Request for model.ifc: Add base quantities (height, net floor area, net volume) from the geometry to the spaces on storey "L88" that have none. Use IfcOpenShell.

First a look at what the model holds.

```python
import ifcopenshell
import ifcopenshell.util.element
import ifcopenshell.util.unit

model = ifcopenshell.open("model.ifc")
print(model.schema)
for unit_type in ("LENGTHUNIT", "AREAUNIT", "VOLUMEUNIT"):
    print(unit_type, ifcopenshell.util.unit.calculate_unit_scale(model, unit_type))
storey = next(s for s in model.by_type("IfcBuildingStorey") if s.Name == "L88")
spaces = [e for e in ifcopenshell.util.element.get_decomposition(storey) if e.is_a("IfcSpace")]
for e in sorted(spaces, key=lambda e: e.id()):
    print(e.id(), e.is_a(), e.Name, list(ifcopenshell.util.element.get_psets(e, qtos_only=True)), sep=" | ")
```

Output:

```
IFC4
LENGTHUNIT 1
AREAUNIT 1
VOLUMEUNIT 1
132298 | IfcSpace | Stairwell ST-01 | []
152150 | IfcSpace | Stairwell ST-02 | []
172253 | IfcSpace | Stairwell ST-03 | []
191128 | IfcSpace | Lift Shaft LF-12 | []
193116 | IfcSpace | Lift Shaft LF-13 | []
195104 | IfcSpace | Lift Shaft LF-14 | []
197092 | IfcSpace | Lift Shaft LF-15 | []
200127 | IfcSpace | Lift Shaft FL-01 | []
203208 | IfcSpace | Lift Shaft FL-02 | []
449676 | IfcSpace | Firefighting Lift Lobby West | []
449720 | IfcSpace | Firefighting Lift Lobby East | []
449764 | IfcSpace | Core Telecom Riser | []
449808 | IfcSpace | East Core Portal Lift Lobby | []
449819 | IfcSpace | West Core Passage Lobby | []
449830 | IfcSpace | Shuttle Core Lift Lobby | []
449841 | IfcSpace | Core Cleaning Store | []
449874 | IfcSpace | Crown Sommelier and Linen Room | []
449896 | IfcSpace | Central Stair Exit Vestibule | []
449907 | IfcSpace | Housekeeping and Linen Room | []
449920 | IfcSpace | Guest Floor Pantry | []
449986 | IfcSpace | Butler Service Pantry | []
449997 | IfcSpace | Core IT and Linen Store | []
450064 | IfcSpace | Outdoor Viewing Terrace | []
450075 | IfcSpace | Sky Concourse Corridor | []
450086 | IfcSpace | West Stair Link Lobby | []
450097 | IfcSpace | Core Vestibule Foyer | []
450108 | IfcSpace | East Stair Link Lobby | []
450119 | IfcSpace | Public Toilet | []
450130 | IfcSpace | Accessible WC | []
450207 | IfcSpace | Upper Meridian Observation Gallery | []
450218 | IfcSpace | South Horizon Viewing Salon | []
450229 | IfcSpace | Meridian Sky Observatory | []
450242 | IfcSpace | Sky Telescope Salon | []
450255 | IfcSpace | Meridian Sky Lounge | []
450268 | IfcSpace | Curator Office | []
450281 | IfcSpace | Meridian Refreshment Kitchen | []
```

```python
import ifcopenshell
import ifcopenshell.api.pset
import ifcopenshell.geom
import ifcopenshell.util.element
import ifcopenshell.util.shape
import ifcopenshell.util.unit

model = ifcopenshell.open("model.ifc")
unit_scale = ifcopenshell.util.unit.calculate_unit_scale(model)
area_scale = ifcopenshell.util.unit.calculate_unit_scale(model, "AREAUNIT")
volume_scale = ifcopenshell.util.unit.calculate_unit_scale(model, "VOLUMEUNIT")
settings = ifcopenshell.geom.settings()

storey = next(s for s in model.by_type("IfcBuildingStorey") if s.Name == "L88")
spaces = [e for e in ifcopenshell.util.element.get_decomposition(storey) if e.is_a("IfcSpace")]

for e in sorted(spaces, key=lambda e: e.id()):
    if ifcopenshell.util.element.get_psets(e, qtos_only=True, should_inherit=False):
        continue
    # Geometry comes back in metres, in the element's own axes.
    shape = ifcopenshell.geom.create_shape(settings, e)
    values = {
        "Height": ifcopenshell.util.shape.get_z(shape.geometry) / unit_scale,
        "NetFloorArea": ifcopenshell.util.shape.get_footprint_area(shape.geometry) / area_scale,
        "NetVolume": ifcopenshell.util.shape.get_volume(shape.geometry) / volume_scale,
    }
    qto = ifcopenshell.api.pset.add_qto(model, product=e, name="Qto_SpaceBaseQuantities")
    ifcopenshell.api.pset.edit_qto(model, qto=qto, properties=values)
    print(e.id(), {k: round(v, 3) for k, v in values.items()})

model.write("model-out.ifc")
```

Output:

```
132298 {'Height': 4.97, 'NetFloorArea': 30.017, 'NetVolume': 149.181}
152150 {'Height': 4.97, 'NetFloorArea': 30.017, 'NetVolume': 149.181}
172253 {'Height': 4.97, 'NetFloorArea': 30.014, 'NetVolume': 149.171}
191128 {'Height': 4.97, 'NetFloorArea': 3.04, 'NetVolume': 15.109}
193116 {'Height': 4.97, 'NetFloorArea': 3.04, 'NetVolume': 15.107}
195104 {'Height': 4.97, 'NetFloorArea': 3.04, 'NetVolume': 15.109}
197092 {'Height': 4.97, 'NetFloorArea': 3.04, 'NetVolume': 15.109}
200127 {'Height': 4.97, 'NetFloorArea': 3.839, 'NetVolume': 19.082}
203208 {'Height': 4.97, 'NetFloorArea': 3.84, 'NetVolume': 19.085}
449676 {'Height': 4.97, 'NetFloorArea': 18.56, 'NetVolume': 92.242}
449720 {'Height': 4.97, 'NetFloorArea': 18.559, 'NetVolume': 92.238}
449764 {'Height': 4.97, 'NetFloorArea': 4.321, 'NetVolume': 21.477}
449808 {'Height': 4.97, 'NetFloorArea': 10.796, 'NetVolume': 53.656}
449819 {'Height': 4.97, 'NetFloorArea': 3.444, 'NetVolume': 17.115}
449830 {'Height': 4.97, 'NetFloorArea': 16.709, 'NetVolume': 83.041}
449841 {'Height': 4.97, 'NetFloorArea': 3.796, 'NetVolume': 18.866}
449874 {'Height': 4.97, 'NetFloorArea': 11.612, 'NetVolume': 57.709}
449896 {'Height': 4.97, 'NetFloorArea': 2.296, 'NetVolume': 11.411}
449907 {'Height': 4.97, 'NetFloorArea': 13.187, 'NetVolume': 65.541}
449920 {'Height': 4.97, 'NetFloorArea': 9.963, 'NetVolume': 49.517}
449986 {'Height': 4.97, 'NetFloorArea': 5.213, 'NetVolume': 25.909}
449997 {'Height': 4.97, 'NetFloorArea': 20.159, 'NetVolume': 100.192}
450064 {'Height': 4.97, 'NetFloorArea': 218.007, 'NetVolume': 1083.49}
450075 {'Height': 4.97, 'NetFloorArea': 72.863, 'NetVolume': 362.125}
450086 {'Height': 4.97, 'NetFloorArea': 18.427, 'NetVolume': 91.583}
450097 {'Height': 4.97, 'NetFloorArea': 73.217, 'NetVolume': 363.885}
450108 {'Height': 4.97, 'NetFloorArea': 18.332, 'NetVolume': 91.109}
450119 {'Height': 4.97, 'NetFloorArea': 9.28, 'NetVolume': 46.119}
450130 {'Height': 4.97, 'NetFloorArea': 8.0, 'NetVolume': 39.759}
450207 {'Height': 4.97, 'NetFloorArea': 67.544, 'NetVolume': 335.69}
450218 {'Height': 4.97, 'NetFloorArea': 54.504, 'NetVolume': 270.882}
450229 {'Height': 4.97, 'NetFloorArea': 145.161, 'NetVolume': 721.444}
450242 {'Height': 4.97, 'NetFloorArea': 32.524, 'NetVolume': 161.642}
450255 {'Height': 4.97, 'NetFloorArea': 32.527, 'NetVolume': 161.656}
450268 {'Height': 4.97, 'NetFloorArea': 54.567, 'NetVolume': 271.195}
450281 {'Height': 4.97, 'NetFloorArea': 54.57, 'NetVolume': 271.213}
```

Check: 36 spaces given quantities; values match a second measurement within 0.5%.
